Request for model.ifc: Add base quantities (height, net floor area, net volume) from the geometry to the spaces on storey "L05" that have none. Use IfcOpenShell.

First a look at what the model holds.

```python
import ifcopenshell
import ifcopenshell.util.element
import ifcopenshell.util.unit

model = ifcopenshell.open("model.ifc")
print(model.schema)
for unit_type in ("LENGTHUNIT", "AREAUNIT", "VOLUMEUNIT"):
    print(unit_type, ifcopenshell.util.unit.calculate_unit_scale(model, unit_type))
storey = next(s for s in model.by_type("IfcBuildingStorey") if s.Name == "L05")
spaces = [e for e in ifcopenshell.util.element.get_decomposition(storey) if e.is_a("IfcSpace")]
for e in sorted(spaces, key=lambda e: e.id()):
    print(e.id(), e.is_a(), e.Name, list(ifcopenshell.util.element.get_psets(e, qtos_only=True)), sep=" | ")
```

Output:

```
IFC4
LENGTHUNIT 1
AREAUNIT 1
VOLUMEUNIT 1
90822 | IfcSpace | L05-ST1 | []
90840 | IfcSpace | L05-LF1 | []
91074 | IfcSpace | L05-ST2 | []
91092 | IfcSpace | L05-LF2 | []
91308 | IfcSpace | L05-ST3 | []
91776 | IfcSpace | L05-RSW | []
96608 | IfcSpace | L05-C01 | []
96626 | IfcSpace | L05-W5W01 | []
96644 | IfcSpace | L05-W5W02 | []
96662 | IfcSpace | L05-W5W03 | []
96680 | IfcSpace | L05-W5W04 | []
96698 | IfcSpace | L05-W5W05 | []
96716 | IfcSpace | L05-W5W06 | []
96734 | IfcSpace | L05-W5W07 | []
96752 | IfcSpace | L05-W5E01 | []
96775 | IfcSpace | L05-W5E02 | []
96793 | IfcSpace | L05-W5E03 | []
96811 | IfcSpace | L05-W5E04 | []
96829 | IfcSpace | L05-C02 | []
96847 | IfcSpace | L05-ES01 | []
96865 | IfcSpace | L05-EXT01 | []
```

```python
import ifcopenshell
import ifcopenshell.api.pset
import ifcopenshell.geom
import ifcopenshell.util.element
import ifcopenshell.util.shape
import ifcopenshell.util.unit

model = ifcopenshell.open("model.ifc")
unit_scale = ifcopenshell.util.unit.calculate_unit_scale(model)
area_scale = ifcopenshell.util.unit.calculate_unit_scale(model, "AREAUNIT")
volume_scale = ifcopenshell.util.unit.calculate_unit_scale(model, "VOLUMEUNIT")
settings = ifcopenshell.geom.settings()

storey = next(s for s in model.by_type("IfcBuildingStorey") if s.Name == "L05")
spaces = [e for e in ifcopenshell.util.element.get_decomposition(storey) if e.is_a("IfcSpace")]

for e in sorted(spaces, key=lambda e: e.id()):
    if ifcopenshell.util.element.get_psets(e, qtos_only=True, should_inherit=False):
        continue
    # Geometry comes back in metres, in the element's own axes.
    shape = ifcopenshell.geom.create_shape(settings, e)
    values = {
        "Height": ifcopenshell.util.shape.get_z(shape.geometry) / unit_scale,
        "NetFloorArea": ifcopenshell.util.shape.get_footprint_area(shape.geometry) / area_scale,
        "NetVolume": ifcopenshell.util.shape.get_volume(shape.geometry) / volume_scale,
    }
    qto = ifcopenshell.api.pset.add_qto(model, product=e, name="Qto_SpaceBaseQuantities")
    ifcopenshell.api.pset.edit_qto(model, qto=qto, properties=values)
    print(e.id(), {k: round(v, 3) for k, v in values.items()})

model.write("model-out.ifc")
```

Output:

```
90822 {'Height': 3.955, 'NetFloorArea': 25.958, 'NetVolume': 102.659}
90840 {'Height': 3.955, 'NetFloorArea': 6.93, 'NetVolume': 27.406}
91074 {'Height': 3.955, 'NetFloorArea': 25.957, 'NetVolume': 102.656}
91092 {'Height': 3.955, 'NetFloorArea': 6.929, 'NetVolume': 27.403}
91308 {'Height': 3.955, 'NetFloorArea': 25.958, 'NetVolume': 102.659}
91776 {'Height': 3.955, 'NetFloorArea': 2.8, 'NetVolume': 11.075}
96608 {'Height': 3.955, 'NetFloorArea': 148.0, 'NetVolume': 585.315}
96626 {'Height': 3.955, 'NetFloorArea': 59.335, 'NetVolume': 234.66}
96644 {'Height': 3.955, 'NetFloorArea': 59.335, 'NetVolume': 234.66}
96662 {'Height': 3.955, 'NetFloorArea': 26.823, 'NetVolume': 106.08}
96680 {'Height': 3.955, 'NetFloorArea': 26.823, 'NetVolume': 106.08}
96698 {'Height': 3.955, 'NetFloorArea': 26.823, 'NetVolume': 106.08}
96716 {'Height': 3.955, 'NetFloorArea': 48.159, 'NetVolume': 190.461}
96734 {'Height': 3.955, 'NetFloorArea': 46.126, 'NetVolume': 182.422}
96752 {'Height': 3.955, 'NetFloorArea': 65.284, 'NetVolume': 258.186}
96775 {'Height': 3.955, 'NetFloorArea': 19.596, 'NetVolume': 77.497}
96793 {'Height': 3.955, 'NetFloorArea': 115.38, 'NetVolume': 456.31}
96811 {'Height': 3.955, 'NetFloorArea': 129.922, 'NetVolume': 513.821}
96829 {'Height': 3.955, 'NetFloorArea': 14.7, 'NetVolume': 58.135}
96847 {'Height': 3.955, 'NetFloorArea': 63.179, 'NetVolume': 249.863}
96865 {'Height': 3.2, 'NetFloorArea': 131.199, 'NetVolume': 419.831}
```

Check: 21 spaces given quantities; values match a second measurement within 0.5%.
